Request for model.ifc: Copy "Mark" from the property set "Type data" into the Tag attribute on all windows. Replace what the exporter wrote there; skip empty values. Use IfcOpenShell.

First a look at what the model holds.

```python
import ifcopenshell
import ifcopenshell.util.element

model = ifcopenshell.open("model.ifc")
print(model.schema)
windows = model.by_type("IfcWindow")
print(len(windows), "windows")
for e in windows[:8]:
    source = ifcopenshell.util.element.get_pset(e, "Type data", "Mark")
    target = e.Tag
    print(e.id(), repr(source), repr(target), sep=" | ")
```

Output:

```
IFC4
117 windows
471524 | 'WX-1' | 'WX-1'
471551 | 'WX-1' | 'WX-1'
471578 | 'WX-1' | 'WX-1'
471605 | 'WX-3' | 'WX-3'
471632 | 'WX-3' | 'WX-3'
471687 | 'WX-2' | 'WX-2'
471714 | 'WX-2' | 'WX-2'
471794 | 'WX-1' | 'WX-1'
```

```python
import ifcopenshell
import ifcopenshell.util.element

model = ifcopenshell.open("model.ifc")

count = 0
for e in model.by_type("IfcWindow"):
    value = ifcopenshell.util.element.get_pset(e, "Type data", "Mark")
    current = e.Tag
    if not value or not value.strip() or current == value:
        continue
    e.Tag = value
    count += 1

print(count, "windows updated")

model.write("model_edited.ifc")
```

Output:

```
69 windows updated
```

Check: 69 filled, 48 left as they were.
